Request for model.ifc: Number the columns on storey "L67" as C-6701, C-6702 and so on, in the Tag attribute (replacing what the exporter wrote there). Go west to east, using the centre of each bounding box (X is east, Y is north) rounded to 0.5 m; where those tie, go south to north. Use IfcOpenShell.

First a look at what the model holds.

```python
import ifcopenshell
import ifcopenshell.util.element
import ifcopenshell.util.placement

model = ifcopenshell.open("model.ifc")
print(model.schema)
storey = next(s for s in model.by_type("IfcBuildingStorey") if s.Name == "L67")
columns = [e for e in ifcopenshell.util.element.get_decomposition(storey) if e.is_a("IfcColumn")]
for e in sorted(columns, key=lambda e: e.id()):
    origin = ifcopenshell.util.placement.get_local_placement(e.ObjectPlacement)[:3, 3]
    print(e.id(), e.Tag, e.Name, origin.round(2) + 0.0, sep=" | ")
```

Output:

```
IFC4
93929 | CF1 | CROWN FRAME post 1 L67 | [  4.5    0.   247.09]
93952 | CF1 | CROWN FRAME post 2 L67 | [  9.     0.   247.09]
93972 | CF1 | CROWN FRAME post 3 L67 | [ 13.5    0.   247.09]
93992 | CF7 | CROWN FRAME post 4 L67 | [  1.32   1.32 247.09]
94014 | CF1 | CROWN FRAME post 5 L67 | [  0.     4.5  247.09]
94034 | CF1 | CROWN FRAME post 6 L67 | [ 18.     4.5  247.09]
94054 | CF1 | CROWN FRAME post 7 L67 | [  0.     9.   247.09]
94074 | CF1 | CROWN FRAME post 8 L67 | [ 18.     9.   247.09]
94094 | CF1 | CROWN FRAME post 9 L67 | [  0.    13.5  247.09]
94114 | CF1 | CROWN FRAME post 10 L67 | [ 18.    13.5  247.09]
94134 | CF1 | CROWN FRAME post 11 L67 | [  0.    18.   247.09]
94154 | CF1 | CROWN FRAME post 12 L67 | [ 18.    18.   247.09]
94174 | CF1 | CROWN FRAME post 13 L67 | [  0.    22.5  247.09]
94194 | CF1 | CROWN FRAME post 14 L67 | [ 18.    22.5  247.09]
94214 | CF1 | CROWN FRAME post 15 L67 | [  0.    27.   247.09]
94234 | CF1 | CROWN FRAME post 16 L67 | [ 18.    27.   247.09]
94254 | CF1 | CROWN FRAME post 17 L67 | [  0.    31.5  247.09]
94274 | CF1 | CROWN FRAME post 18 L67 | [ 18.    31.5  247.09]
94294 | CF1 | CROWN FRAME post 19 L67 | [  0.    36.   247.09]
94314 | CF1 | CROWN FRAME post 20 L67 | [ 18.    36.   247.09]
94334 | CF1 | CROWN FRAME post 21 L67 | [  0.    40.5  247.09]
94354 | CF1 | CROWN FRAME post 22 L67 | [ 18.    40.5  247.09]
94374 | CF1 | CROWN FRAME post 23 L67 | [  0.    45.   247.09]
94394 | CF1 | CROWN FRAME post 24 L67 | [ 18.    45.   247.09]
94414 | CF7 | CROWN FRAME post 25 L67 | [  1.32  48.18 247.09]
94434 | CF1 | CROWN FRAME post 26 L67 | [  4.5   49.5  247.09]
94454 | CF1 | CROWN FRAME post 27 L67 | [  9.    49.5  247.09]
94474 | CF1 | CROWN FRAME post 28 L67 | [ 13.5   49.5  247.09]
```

```python
import ifcopenshell
import ifcopenshell.geom
import ifcopenshell.util.element
import ifcopenshell.util.shape

model = ifcopenshell.open("model.ifc")
settings = ifcopenshell.geom.settings()
settings.set("use-world-coords", True)


def centre(element):
    shape = ifcopenshell.geom.create_shape(settings, element)
    return ifcopenshell.util.shape.get_bbox_centroid(shape.geometry)


storey = next(s for s in model.by_type("IfcBuildingStorey") if s.Name == "L67")
columns = [e for e in ifcopenshell.util.element.get_decomposition(storey) if e.is_a("IfcColumn")]

# Insertion points can sit at a corner or the storey origin, so sort by the geometry (in metres).
centres = {e: centre(e) for e in columns}
columns.sort(key=lambda e: (round(centres[e][0] / 0.5), centres[e][1]))

for i, e in enumerate(columns, start=1):
    number = f"C-67{i:02d}"
    e.Tag = number
    print(e.id(), number)

model.write("model-out.ifc")
```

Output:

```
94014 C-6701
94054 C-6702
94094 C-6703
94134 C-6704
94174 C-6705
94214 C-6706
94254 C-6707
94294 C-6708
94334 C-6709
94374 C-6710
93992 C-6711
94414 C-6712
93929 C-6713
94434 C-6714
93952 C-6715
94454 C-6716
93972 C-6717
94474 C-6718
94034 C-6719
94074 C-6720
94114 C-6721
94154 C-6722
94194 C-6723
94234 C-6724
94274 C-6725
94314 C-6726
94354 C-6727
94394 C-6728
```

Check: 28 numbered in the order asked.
